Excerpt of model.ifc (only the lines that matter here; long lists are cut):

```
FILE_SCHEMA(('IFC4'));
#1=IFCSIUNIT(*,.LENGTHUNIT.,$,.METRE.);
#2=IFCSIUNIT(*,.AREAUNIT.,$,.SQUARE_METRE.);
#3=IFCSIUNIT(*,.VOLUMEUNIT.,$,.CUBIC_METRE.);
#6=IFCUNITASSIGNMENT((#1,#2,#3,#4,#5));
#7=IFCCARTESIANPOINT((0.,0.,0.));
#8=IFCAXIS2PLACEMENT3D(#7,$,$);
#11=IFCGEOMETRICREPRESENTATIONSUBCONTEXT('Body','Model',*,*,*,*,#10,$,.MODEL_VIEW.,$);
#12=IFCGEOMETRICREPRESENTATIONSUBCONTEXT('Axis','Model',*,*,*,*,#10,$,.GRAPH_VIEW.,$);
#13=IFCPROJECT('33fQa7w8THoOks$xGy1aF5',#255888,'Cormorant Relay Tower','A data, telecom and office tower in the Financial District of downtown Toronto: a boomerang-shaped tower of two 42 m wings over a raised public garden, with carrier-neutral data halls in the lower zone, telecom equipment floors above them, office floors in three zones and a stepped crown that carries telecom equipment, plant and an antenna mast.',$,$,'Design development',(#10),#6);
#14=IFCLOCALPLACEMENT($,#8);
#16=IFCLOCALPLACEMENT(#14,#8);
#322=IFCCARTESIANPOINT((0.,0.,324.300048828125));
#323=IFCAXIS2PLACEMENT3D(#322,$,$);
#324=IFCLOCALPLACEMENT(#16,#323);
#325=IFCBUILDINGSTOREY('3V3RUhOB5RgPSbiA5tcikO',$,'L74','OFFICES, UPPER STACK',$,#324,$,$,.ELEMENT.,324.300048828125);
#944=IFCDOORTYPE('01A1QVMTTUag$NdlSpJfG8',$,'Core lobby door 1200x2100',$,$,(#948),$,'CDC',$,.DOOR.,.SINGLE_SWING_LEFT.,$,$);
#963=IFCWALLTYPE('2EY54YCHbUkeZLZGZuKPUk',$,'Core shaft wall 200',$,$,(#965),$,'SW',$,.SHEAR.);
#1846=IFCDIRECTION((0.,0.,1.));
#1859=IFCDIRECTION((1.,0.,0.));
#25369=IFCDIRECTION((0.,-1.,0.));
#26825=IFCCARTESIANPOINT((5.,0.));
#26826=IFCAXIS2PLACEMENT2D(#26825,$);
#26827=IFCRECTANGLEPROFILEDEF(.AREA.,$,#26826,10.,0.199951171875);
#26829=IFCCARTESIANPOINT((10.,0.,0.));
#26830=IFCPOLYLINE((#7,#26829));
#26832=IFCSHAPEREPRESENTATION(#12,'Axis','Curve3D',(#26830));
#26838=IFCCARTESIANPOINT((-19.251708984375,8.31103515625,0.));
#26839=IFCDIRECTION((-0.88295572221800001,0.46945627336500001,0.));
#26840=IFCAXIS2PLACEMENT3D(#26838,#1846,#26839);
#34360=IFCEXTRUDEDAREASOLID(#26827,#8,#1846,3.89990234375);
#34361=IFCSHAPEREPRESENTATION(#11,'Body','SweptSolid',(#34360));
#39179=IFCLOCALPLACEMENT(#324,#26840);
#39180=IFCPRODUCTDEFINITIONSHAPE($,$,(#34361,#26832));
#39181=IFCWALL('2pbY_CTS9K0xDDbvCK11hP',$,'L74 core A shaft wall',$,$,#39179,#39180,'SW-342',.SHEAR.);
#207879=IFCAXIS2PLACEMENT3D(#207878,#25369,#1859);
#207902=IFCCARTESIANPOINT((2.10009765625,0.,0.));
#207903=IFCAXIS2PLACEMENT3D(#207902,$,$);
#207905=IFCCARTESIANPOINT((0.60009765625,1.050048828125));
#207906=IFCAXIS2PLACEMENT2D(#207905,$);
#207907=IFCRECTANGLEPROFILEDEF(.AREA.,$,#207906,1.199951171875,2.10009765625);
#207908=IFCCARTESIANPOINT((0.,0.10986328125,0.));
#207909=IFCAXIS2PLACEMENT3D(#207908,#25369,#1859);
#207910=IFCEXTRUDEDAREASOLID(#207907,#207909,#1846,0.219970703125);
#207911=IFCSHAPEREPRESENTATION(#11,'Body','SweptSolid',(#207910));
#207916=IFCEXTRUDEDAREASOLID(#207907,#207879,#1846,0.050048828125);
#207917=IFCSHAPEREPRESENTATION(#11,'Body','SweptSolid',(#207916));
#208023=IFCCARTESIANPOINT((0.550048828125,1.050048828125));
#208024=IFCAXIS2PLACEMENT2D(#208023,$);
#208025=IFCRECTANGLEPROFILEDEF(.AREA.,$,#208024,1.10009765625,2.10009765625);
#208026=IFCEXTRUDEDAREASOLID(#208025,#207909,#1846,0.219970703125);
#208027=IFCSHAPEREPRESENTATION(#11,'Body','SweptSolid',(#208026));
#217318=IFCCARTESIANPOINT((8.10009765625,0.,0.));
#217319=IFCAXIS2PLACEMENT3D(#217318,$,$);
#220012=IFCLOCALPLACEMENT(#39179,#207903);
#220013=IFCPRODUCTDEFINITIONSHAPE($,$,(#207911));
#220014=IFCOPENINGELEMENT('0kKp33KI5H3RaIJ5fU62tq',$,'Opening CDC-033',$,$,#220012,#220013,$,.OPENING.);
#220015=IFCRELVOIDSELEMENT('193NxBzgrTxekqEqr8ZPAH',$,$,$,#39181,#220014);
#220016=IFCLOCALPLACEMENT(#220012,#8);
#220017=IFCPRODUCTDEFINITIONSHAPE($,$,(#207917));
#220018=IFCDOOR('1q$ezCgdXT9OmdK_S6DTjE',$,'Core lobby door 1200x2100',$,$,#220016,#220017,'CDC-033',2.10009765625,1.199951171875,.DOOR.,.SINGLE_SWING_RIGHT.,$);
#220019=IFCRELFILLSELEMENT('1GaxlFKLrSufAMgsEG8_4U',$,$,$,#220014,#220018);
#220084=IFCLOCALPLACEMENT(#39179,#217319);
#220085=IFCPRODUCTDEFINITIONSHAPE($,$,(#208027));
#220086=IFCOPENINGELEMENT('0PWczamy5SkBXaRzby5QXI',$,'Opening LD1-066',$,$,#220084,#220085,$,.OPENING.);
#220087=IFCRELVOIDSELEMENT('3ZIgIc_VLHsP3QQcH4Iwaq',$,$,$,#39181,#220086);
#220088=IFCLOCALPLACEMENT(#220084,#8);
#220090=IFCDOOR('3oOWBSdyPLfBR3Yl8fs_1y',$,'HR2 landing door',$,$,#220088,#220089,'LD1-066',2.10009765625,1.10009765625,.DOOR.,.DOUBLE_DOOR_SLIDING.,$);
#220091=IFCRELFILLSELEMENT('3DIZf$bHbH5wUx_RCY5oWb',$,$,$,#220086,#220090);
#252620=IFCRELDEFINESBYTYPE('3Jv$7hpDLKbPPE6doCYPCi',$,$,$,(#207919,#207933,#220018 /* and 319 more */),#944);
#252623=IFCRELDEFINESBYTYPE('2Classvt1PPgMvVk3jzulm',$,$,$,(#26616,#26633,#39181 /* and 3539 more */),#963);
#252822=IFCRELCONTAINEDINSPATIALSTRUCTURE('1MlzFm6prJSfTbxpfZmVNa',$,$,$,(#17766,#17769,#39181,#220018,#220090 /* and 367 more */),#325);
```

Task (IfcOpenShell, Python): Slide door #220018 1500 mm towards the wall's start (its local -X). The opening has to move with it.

```python
import ifcopenshell
import ifcopenshell.api.geometry
import ifcopenshell.util.placement
import ifcopenshell.util.unit

model = ifcopenshell.open("model.ifc")
unit_scale = ifcopenshell.util.unit.calculate_unit_scale(model)

door = model.by_guid("1q$ezCgdXT9OmdK_S6DTjE")
opening = door.FillsVoids[0].RelatingOpeningElement
wall = opening.VoidsElements[0].RelatingBuildingElement

wall_matrix = ifcopenshell.util.placement.get_local_placement(wall.ObjectPlacement)
shift = wall_matrix[:3, 0] * -1.5 / unit_scale
before = ifcopenshell.util.placement.get_local_placement(door.ObjectPlacement)[:3, 3].copy()

# The door is placed relative to its opening, so it follows when the opening moves.
matrix = ifcopenshell.util.placement.get_local_placement(opening.ObjectPlacement)
matrix[:3, 3] += shift
ifcopenshell.api.geometry.edit_object_placement(
    model, product=opening, matrix=matrix, is_si=False, should_transform_children=True
)

after = ifcopenshell.util.placement.get_local_placement(door.ObjectPlacement)[:3, 3]
print("door moved by", (after - before).round(3) + 0.0)

model.write("model_edited.ifc")
```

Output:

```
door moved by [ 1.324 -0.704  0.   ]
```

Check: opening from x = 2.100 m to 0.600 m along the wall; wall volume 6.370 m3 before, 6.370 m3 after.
